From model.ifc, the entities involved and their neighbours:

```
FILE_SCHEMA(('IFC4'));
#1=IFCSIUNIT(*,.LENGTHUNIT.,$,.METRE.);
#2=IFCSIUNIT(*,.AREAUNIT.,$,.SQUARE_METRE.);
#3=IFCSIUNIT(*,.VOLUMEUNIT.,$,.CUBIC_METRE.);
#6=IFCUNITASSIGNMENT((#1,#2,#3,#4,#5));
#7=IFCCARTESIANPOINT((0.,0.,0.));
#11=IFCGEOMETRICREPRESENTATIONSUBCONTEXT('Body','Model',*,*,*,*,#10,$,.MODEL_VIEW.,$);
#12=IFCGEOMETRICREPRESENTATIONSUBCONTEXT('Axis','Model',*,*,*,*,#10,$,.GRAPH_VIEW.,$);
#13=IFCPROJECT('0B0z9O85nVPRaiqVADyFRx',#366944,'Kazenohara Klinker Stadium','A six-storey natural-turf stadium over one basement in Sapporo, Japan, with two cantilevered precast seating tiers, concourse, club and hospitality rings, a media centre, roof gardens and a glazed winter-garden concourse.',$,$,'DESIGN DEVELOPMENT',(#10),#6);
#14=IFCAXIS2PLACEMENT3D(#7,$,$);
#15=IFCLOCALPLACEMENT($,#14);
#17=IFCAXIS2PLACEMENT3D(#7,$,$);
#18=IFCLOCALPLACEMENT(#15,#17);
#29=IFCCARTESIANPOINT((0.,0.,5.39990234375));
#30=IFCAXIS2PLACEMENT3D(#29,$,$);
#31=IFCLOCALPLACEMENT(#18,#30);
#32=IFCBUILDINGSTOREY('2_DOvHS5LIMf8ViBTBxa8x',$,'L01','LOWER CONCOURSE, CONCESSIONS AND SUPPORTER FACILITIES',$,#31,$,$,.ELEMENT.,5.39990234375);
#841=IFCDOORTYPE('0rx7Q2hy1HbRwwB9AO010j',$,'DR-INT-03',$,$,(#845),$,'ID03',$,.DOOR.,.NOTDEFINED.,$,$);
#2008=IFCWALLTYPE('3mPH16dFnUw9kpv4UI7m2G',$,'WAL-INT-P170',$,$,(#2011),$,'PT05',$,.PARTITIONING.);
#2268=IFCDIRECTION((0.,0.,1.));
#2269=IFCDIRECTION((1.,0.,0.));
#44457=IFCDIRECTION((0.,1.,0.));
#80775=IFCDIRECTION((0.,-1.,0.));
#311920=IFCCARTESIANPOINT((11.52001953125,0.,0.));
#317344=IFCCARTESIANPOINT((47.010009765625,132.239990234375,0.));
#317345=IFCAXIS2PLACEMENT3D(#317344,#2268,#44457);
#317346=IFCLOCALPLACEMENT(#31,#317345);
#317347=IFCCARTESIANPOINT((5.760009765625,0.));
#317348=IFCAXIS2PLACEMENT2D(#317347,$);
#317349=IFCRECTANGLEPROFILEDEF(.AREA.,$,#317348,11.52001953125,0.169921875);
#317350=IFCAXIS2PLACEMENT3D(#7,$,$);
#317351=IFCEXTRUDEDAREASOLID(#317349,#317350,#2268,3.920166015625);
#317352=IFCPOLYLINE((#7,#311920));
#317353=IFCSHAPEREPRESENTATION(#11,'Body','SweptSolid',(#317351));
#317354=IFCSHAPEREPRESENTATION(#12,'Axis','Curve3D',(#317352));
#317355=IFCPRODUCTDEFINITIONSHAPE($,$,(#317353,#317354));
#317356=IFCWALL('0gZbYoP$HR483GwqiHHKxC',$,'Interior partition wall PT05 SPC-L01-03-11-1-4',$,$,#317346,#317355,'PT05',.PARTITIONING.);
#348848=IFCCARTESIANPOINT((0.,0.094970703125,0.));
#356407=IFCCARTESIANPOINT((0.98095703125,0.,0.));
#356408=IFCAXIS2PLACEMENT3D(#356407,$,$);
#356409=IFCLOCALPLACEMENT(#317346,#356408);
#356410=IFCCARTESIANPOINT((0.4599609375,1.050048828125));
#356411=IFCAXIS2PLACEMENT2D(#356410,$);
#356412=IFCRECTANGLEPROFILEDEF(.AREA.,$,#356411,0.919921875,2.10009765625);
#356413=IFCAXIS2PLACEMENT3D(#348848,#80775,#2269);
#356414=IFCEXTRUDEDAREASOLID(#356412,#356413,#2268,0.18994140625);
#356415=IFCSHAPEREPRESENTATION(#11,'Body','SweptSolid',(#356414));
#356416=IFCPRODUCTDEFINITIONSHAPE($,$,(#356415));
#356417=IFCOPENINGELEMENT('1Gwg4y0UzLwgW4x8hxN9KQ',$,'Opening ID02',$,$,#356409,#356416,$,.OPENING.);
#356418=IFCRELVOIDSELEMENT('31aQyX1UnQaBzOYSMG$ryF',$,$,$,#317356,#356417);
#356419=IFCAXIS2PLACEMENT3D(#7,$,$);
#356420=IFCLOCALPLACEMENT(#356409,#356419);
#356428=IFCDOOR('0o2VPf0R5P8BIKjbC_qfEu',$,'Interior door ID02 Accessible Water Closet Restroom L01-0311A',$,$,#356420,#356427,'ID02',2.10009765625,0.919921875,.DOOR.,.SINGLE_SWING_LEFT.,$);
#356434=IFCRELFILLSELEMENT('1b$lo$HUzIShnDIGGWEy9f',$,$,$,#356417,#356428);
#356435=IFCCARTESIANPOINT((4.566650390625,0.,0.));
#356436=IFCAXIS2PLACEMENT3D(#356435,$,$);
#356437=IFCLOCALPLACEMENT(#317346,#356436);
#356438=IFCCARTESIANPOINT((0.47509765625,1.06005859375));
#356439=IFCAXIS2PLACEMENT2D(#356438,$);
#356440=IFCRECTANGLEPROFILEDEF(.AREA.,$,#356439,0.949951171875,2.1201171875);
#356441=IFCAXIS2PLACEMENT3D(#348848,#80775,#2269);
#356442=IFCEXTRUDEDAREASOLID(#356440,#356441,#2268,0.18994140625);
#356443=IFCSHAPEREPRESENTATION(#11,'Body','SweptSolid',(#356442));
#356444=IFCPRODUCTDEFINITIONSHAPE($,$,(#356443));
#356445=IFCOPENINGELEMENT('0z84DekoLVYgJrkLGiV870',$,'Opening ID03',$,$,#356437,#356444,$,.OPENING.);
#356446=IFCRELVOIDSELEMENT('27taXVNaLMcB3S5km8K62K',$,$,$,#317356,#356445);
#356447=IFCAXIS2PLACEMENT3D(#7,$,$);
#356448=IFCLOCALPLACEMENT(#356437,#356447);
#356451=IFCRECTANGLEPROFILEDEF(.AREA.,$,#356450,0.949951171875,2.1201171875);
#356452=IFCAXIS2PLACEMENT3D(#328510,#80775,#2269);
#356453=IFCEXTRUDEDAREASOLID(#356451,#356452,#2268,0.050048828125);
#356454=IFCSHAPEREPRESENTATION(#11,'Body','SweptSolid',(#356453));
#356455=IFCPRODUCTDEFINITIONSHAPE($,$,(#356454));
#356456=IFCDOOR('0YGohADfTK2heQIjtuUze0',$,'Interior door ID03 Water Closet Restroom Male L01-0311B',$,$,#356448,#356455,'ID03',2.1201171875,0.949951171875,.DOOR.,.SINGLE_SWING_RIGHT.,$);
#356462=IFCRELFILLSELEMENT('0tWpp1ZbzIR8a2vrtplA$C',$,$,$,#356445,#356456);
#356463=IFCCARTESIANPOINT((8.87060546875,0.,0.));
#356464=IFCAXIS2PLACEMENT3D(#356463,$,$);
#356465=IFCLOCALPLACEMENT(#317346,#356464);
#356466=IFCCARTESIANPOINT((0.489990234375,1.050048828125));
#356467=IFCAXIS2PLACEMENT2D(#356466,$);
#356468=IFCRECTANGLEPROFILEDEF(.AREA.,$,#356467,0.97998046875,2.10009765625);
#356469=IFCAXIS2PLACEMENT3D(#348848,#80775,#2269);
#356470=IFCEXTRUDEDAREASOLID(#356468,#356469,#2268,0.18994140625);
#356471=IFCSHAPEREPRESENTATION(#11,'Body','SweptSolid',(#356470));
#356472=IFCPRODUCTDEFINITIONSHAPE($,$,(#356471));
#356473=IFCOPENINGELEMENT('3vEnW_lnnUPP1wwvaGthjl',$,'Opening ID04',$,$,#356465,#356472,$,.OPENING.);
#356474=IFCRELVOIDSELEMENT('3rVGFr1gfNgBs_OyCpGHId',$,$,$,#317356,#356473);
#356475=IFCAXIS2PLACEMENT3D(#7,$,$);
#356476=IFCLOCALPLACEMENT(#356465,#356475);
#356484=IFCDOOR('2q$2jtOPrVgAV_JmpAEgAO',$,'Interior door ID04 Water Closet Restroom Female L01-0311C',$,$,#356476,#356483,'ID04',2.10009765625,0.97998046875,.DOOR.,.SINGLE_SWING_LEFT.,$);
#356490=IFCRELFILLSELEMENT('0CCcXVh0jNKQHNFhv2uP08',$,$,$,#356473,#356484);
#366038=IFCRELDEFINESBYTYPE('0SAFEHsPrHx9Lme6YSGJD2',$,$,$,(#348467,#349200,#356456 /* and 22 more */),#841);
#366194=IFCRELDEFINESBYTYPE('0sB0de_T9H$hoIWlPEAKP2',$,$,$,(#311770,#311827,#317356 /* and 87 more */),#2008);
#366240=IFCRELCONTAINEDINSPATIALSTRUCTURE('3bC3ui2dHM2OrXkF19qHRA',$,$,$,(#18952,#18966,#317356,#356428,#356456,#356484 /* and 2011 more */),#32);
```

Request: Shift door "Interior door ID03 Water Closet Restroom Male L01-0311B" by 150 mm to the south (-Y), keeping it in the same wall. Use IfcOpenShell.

```python
import ifcopenshell
import ifcopenshell.api.geometry
import ifcopenshell.util.placement

model = ifcopenshell.open("model.ifc")

door = model.by_guid("0YGohADfTK2heQIjtuUze0")
opening = door.FillsVoids[0].RelatingOpeningElement
wall = opening.VoidsElements[0].RelatingBuildingElement

wall_matrix = ifcopenshell.util.placement.get_local_placement(wall.ObjectPlacement)
shift = wall_matrix[:3, 0] * -0.15
before = ifcopenshell.util.placement.get_local_placement(door.ObjectPlacement)[:3, 3].copy()

# The door is placed relative to its opening, so it follows when the opening moves.
matrix = ifcopenshell.util.placement.get_local_placement(opening.ObjectPlacement)
matrix[:3, 3] += shift
ifcopenshell.api.geometry.edit_object_placement(
    model, product=opening, matrix=matrix, is_si=False, should_transform_children=True
)

after = ifcopenshell.util.placement.get_local_placement(door.ObjectPlacement)[:3, 3]
print("door moved by", (after - before).round(3) + 0.0)

model.write("model_edited.ifc")
```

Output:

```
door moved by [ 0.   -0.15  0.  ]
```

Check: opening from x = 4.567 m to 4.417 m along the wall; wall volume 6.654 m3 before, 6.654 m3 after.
